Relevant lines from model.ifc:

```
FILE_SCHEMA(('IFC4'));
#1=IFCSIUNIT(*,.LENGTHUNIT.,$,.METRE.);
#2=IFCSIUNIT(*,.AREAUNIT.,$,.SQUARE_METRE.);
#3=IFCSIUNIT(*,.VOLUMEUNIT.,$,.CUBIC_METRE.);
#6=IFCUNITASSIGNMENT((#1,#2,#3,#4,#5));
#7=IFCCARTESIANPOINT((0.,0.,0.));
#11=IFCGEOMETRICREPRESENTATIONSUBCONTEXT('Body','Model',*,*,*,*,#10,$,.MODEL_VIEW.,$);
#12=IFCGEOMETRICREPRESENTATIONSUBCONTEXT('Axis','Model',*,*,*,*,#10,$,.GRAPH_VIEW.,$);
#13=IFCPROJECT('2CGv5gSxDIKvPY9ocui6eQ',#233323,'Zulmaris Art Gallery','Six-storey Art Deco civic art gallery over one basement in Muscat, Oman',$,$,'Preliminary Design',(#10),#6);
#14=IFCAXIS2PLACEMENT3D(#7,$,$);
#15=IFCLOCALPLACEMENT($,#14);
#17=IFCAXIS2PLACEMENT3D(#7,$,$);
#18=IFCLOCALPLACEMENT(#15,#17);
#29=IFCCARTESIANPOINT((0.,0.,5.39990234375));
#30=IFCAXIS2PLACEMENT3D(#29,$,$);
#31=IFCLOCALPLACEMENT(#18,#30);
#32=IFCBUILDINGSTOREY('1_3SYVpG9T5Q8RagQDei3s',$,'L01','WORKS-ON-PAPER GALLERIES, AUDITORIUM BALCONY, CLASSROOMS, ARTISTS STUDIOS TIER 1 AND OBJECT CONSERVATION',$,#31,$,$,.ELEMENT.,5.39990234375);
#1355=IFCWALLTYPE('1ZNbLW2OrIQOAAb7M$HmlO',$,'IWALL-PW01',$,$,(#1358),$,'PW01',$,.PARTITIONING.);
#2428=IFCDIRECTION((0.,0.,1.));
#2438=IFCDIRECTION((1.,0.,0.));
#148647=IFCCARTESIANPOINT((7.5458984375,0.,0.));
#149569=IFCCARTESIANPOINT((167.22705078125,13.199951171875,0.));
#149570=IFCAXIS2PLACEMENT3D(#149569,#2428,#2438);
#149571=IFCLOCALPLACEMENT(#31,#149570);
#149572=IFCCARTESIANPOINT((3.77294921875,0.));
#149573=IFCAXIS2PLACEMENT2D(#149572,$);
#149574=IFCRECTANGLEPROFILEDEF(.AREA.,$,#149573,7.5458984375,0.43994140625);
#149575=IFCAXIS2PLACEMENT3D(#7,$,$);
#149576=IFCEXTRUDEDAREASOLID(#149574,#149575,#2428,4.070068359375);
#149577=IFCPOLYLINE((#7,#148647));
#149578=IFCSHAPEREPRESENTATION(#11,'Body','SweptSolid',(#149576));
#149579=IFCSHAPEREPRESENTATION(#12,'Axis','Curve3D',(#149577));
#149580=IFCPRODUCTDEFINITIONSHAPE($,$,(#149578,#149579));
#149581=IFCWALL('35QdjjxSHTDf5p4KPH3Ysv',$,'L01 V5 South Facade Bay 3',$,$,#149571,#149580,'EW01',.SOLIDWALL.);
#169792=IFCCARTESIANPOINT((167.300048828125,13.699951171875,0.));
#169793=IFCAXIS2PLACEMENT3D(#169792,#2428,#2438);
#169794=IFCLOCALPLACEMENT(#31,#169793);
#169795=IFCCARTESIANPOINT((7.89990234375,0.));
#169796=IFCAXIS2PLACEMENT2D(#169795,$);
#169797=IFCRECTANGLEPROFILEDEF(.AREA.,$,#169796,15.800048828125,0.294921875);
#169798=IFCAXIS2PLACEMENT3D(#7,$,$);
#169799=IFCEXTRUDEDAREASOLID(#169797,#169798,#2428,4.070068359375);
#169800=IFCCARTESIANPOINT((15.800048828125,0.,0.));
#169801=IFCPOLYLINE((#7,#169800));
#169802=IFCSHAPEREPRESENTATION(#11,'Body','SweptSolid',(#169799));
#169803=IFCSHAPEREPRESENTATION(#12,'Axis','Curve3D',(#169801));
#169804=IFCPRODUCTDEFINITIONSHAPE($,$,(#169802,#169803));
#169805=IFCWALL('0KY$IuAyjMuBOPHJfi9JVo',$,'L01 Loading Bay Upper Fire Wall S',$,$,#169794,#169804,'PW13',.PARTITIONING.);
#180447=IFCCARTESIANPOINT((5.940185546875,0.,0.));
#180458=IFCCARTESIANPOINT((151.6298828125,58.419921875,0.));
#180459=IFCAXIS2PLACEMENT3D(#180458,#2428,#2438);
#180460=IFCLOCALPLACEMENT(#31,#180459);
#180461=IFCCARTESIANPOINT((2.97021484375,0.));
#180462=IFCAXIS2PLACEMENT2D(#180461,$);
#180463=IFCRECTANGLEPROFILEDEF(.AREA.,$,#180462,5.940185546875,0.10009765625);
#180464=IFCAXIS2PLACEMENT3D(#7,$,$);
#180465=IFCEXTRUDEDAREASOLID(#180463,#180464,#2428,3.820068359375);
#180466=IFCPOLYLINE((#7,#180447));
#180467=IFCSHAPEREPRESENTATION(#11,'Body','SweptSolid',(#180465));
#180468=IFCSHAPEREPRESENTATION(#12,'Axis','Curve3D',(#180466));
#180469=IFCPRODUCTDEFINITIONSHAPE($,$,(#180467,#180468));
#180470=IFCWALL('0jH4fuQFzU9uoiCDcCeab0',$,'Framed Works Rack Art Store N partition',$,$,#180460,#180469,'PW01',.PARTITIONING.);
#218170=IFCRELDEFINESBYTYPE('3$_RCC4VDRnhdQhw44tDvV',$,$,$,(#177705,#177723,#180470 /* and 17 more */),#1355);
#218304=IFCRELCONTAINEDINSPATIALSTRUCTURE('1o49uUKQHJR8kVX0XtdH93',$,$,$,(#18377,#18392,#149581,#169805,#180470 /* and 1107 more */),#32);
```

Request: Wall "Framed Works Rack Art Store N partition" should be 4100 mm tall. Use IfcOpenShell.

```python
import ifcopenshell
import ifcopenshell.geom
import ifcopenshell.util.representation
import ifcopenshell.util.shape
import ifcopenshell.util.unit

model = ifcopenshell.open("model.ifc")
unit_scale = ifcopenshell.util.unit.calculate_unit_scale(model)
settings = ifcopenshell.geom.settings()


def volume(element):
    """Net volume in cubic metres, openings subtracted."""
    shape = ifcopenshell.geom.create_shape(settings, element)
    return ifcopenshell.util.shape.get_volume(shape.geometry)


wall = model.by_id(180470)
before = volume(wall)

body = ifcopenshell.util.representation.get_representation(wall, "Model", "Body")
solid = body.Items[0]
old_height = solid.Depth
solid.Depth = 4.1 / unit_scale
after = volume(wall)

print(f"height {old_height:g} -> {solid.Depth:g}, volume {before:.3f} -> {after:.3f} m3")

model.write("model_rev.ifc")
```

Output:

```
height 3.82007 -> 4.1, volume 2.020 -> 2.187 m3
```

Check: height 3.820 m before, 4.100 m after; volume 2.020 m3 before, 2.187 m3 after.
